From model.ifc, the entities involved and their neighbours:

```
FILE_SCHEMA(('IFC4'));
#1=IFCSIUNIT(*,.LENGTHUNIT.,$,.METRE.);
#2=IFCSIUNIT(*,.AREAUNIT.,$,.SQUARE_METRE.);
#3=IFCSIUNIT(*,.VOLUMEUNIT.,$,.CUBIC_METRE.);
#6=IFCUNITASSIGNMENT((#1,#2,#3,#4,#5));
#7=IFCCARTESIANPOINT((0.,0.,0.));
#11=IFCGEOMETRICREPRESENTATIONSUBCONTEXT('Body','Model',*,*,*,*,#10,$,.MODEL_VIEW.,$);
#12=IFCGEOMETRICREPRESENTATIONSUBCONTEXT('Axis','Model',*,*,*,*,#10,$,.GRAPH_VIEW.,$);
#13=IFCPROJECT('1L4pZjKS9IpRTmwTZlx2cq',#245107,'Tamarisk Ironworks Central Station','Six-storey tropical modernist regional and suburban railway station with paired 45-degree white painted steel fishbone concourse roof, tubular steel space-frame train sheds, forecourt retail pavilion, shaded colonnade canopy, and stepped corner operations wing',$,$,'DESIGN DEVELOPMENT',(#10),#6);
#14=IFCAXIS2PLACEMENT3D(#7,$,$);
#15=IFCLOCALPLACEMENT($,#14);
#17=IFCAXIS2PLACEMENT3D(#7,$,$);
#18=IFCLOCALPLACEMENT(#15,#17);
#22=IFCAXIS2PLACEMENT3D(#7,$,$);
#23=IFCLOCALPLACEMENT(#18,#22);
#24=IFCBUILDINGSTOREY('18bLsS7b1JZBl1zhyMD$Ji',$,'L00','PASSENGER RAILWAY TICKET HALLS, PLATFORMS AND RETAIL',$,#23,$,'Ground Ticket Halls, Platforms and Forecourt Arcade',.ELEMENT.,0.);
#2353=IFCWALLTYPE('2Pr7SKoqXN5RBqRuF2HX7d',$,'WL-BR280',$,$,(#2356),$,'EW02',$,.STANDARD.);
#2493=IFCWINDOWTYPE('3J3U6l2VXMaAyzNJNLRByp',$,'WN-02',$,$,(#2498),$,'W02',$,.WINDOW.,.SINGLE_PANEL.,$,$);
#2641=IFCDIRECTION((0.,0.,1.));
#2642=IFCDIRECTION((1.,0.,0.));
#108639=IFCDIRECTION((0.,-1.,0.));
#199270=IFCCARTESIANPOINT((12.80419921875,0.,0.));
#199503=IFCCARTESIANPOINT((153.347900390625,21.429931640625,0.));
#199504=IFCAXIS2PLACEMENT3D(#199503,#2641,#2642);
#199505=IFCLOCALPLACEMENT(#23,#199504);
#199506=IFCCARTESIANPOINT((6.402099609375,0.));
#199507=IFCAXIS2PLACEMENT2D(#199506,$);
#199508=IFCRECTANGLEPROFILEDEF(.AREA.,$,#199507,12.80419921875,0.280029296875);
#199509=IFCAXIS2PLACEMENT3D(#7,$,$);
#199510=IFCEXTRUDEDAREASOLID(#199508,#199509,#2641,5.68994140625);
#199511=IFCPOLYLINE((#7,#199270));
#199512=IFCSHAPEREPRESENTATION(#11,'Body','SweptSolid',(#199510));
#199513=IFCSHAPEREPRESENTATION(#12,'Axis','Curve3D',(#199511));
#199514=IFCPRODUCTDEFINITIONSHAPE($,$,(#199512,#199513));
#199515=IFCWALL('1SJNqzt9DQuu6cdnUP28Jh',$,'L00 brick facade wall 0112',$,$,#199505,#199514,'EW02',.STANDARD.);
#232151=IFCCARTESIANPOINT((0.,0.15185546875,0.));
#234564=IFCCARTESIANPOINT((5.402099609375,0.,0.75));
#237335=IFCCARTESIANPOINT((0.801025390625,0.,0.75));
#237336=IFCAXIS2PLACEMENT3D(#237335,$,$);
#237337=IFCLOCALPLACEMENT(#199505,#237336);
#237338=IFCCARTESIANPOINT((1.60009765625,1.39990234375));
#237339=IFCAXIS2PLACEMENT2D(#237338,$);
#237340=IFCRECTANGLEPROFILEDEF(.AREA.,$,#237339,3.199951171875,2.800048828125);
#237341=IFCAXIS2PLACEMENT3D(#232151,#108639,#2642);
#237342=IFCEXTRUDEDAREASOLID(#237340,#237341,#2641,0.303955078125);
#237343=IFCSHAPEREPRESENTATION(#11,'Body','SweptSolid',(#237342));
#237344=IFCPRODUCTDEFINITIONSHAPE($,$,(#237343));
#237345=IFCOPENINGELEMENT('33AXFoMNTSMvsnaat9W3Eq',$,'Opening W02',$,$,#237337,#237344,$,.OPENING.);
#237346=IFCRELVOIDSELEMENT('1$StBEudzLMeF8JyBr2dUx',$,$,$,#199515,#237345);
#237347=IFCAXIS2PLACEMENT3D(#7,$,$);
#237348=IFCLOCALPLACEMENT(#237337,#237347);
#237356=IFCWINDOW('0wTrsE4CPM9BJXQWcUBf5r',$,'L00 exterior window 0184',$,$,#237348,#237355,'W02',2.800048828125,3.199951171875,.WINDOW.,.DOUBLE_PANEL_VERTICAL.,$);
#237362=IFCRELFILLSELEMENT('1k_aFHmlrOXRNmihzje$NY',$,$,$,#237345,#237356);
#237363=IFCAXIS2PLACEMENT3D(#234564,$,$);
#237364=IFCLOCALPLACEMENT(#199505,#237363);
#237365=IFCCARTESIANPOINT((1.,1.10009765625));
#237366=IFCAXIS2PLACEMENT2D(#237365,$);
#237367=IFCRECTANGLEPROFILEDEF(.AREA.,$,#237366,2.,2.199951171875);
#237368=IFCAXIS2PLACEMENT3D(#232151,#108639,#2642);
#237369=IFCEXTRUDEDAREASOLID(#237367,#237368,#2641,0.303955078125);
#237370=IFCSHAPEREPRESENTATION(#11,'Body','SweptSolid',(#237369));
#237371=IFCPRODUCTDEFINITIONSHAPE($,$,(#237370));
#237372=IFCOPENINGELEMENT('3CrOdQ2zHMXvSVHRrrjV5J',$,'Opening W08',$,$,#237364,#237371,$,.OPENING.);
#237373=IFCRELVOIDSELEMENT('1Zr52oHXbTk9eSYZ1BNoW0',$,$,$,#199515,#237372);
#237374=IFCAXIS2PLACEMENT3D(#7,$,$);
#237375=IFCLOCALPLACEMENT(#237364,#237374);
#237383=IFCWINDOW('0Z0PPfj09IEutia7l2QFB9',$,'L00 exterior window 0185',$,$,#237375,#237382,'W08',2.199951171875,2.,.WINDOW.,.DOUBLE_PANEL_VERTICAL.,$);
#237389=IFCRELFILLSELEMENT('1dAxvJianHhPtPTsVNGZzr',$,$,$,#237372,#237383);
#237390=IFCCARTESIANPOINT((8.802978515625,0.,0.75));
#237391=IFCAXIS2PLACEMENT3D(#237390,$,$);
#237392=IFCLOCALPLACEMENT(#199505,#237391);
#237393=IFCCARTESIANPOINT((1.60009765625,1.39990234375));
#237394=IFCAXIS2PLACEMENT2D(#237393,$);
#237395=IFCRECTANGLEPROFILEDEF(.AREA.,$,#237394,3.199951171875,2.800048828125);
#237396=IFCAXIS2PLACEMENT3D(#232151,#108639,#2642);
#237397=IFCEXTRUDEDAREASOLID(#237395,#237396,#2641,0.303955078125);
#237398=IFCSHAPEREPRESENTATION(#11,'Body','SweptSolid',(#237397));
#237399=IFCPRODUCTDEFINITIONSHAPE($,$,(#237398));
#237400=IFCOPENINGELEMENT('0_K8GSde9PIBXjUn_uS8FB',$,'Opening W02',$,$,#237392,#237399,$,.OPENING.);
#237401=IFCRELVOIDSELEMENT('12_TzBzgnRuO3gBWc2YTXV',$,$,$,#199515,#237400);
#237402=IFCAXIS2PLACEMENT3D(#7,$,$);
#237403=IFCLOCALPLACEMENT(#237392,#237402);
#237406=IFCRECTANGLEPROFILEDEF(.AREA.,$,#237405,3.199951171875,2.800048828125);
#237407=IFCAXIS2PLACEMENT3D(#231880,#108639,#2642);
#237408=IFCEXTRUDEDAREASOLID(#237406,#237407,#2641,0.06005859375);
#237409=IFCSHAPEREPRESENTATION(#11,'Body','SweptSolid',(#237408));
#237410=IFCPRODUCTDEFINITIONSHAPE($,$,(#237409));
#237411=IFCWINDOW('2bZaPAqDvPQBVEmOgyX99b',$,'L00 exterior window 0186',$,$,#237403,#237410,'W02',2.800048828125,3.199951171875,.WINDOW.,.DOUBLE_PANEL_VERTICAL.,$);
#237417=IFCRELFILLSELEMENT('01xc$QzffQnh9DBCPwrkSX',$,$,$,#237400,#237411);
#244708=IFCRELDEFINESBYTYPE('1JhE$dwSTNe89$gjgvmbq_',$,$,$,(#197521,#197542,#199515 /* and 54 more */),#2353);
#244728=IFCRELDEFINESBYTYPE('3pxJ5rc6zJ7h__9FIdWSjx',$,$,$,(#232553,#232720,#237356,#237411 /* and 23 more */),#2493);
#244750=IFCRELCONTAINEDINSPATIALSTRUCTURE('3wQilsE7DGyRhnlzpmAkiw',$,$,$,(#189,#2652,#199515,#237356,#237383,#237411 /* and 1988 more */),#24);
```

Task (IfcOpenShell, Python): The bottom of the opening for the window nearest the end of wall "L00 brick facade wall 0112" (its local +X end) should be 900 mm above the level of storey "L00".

```python
import numpy as np
import ifcopenshell
import ifcopenshell.api.geometry
import ifcopenshell.geom
import ifcopenshell.util.element
import ifcopenshell.util.placement
import ifcopenshell.util.shape
import ifcopenshell.util.unit

model = ifcopenshell.open("model.ifc")
unit_scale = ifcopenshell.util.unit.calculate_unit_scale(model)

window = model.by_guid("2bZaPAqDvPQBVEmOgyX99b")
opening = window.FillsVoids[0].RelatingOpeningElement
storey = ifcopenshell.util.element.get_container(window, ifc_class="IfcBuildingStorey")
level = ifcopenshell.util.placement.get_local_placement(storey.ObjectPlacement)[2, 3]

# The opening's origin need not be at the sill, so measure its lowest point.
shape = ifcopenshell.geom.create_shape(ifcopenshell.geom.settings(), opening)
bottom = ifcopenshell.util.shape.get_shape_bottom_elevation(shape, shape.geometry) / unit_scale
dz = level + 0.9 - bottom

shift = np.array([0.0, 0.0, dz])
# The window is placed relative to its opening, so it follows when the opening moves.
matrix = ifcopenshell.util.placement.get_local_placement(opening.ObjectPlacement)
matrix[:3, 3] += shift
ifcopenshell.api.geometry.edit_object_placement(
    model, product=opening, matrix=matrix, is_si=False, should_transform_children=True
)

print(f"moved by {dz * unit_scale:+.3f} m")

model.write("model-out.ifc")
```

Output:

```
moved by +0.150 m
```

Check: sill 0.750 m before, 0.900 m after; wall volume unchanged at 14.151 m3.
